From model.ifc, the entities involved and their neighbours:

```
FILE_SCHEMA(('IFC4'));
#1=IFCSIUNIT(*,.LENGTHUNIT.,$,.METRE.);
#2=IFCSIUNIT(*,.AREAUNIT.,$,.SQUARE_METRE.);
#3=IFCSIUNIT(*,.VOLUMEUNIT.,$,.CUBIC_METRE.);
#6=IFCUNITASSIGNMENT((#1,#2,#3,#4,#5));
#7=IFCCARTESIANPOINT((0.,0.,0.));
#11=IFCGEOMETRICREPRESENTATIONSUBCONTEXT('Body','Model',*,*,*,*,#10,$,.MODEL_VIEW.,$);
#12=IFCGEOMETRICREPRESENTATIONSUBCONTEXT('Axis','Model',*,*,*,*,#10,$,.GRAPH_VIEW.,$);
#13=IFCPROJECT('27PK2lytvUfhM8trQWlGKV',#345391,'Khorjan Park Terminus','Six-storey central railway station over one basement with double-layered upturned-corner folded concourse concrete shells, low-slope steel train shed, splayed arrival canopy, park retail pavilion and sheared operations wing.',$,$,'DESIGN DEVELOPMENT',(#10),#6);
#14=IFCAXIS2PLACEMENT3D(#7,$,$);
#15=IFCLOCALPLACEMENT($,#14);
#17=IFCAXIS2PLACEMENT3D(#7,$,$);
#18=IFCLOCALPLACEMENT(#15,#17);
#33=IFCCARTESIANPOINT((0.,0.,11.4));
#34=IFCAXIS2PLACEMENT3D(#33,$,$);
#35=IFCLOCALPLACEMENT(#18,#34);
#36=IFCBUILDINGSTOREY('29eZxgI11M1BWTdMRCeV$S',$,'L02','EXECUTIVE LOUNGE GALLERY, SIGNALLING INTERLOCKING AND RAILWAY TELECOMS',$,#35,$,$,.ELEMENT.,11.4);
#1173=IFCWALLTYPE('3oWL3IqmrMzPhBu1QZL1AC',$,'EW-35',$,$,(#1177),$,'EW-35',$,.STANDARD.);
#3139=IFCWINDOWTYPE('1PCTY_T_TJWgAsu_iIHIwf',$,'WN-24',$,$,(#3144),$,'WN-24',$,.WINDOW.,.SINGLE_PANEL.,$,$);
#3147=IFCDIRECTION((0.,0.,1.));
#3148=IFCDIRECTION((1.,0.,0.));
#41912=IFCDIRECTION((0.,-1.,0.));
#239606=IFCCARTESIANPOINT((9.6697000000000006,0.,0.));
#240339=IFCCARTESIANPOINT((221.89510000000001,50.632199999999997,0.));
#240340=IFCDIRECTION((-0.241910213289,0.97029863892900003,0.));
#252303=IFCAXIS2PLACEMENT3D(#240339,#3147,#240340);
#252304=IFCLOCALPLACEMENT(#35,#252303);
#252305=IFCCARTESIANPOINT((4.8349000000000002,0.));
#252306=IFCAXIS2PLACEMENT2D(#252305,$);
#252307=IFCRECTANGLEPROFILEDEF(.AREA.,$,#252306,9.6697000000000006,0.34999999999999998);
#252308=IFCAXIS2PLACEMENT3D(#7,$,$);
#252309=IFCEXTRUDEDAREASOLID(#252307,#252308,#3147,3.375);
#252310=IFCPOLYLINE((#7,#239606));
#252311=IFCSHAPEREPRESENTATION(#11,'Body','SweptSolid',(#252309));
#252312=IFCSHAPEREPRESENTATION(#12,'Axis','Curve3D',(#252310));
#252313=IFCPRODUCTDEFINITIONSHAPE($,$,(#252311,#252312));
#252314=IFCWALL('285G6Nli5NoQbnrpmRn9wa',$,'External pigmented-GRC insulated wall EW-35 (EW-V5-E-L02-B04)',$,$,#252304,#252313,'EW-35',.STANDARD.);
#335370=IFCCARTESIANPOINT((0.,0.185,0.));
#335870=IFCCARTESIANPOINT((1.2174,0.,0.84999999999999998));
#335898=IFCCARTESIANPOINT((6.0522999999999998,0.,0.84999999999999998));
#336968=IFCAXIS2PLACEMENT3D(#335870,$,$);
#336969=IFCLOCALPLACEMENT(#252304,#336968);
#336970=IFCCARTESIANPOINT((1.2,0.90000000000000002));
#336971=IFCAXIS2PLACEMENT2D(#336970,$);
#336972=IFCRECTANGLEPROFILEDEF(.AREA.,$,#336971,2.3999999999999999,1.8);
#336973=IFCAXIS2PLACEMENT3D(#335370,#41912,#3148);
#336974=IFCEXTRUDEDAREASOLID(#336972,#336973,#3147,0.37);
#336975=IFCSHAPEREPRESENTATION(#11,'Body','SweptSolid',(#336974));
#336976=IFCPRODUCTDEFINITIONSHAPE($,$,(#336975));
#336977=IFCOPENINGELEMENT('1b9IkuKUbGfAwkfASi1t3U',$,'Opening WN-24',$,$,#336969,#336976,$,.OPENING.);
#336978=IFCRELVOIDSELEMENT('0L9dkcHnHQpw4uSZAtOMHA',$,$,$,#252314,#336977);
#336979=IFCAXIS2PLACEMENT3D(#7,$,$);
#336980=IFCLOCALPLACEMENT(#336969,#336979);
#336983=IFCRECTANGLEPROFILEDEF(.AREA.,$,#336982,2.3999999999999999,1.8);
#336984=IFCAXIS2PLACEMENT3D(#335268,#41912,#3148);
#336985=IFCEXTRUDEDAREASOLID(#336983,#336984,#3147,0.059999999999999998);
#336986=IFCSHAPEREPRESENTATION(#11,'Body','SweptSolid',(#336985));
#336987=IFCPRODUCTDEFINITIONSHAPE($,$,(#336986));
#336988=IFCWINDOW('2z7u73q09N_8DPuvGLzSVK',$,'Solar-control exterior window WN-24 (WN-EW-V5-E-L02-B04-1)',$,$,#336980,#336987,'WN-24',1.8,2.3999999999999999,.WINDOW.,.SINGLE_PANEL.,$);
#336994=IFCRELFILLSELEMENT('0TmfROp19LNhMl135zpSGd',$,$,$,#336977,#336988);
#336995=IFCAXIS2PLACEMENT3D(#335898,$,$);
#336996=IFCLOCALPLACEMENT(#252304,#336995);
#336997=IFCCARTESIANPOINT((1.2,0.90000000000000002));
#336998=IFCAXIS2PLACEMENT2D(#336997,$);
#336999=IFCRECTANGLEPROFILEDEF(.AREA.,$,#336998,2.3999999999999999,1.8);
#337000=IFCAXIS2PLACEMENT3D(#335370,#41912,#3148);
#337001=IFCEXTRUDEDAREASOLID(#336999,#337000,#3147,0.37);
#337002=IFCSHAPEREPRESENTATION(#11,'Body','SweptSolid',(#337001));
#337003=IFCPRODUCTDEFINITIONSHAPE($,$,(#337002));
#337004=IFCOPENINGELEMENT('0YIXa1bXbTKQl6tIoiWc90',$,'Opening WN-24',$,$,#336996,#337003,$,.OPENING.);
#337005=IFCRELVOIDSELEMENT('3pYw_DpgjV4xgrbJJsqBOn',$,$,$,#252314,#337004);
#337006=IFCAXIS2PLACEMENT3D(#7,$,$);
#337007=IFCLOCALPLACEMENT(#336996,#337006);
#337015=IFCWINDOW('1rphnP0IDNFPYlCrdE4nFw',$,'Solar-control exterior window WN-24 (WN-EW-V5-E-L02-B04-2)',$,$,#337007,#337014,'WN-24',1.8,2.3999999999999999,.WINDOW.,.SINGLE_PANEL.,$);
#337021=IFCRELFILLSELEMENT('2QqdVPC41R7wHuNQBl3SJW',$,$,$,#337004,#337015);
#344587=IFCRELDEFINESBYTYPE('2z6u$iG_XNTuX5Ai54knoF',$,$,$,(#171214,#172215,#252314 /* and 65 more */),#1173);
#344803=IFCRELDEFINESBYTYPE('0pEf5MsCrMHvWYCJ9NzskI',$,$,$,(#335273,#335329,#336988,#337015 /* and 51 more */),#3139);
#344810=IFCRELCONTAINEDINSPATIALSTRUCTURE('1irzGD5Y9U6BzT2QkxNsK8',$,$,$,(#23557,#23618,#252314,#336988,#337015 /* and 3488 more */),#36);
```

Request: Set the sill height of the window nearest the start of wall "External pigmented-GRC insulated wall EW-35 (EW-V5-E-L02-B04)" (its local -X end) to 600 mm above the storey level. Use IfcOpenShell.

```python
import numpy as np
import ifcopenshell
import ifcopenshell.api.geometry
import ifcopenshell.geom
import ifcopenshell.util.element
import ifcopenshell.util.placement
import ifcopenshell.util.shape
import ifcopenshell.util.unit

model = ifcopenshell.open("model.ifc")
unit_scale = ifcopenshell.util.unit.calculate_unit_scale(model)

window = model.by_guid("2z7u73q09N_8DPuvGLzSVK")
opening = window.FillsVoids[0].RelatingOpeningElement
storey = ifcopenshell.util.element.get_container(window, ifc_class="IfcBuildingStorey")
level = ifcopenshell.util.placement.get_local_placement(storey.ObjectPlacement)[2, 3]

# The opening's origin need not be at the sill, so measure its lowest point.
shape = ifcopenshell.geom.create_shape(ifcopenshell.geom.settings(), opening)
bottom = ifcopenshell.util.shape.get_shape_bottom_elevation(shape, shape.geometry) / unit_scale
dz = level + 0.6 / unit_scale - bottom

shift = np.array([0.0, 0.0, dz])
# The window is placed relative to its opening, so it follows when the opening moves.
matrix = ifcopenshell.util.placement.get_local_placement(opening.ObjectPlacement)
matrix[:3, 3] += shift
ifcopenshell.api.geometry.edit_object_placement(
    model, product=opening, matrix=matrix, is_si=False, should_transform_children=True
)

print(f"moved by {dz * unit_scale:+.3f} m")

model.write("model_v2.ifc")
```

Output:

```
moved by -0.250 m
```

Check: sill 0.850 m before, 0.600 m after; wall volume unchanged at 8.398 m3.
